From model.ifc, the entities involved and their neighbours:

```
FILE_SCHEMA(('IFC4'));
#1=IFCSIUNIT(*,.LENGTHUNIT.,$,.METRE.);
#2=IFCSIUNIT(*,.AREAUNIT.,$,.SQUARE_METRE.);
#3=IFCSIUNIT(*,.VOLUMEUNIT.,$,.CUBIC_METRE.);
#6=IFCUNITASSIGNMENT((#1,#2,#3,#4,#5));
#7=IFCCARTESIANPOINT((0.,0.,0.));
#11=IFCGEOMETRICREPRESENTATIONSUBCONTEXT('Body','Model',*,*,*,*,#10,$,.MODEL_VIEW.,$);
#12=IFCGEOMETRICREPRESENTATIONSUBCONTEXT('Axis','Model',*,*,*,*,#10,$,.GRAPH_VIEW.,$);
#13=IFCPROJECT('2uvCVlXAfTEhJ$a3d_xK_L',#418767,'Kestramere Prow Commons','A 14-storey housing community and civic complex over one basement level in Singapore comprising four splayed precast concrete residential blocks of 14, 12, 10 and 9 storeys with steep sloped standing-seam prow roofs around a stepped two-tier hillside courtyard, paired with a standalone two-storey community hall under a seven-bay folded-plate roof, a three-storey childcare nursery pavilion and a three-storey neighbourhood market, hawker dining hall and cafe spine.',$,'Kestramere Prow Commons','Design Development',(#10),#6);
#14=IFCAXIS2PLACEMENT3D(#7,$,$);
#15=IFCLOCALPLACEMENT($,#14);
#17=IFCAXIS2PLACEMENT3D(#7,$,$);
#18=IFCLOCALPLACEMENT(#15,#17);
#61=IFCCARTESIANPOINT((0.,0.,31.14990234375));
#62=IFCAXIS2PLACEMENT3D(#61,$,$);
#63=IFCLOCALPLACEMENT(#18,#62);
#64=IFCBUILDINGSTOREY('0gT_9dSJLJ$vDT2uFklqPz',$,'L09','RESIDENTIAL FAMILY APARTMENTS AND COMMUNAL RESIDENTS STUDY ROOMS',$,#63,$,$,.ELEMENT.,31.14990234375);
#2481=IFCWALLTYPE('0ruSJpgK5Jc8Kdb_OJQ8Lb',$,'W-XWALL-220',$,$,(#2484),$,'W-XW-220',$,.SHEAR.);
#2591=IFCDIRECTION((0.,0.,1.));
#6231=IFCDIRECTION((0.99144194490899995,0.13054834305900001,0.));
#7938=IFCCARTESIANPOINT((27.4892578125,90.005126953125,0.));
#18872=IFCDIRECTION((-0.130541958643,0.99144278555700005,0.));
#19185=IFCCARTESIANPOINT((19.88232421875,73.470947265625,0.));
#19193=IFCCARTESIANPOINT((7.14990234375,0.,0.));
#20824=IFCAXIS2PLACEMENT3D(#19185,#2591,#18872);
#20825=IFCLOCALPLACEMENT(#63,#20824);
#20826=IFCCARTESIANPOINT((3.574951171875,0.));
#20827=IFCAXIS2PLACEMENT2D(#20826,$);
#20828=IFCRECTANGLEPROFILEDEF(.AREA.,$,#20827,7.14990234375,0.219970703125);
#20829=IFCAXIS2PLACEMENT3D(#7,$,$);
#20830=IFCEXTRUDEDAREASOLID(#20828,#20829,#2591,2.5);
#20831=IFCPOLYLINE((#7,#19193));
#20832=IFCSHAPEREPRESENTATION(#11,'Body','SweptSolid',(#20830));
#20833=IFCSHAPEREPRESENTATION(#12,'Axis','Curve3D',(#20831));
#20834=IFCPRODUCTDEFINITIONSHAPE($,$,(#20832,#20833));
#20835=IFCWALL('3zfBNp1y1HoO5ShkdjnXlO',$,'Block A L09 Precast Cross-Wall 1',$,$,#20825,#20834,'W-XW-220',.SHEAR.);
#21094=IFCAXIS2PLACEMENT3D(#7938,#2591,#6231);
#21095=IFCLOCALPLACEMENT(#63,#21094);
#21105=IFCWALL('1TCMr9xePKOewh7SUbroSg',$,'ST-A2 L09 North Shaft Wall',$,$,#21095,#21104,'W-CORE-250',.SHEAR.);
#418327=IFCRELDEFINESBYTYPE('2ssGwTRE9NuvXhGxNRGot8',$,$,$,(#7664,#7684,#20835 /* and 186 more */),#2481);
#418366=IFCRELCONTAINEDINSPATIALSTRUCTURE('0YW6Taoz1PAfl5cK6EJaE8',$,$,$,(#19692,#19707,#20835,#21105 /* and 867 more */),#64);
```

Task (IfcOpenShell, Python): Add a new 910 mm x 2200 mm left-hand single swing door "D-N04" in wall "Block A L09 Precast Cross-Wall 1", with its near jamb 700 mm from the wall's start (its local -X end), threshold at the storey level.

```python
import numpy as np
import ifcopenshell
import ifcopenshell.api.feature
import ifcopenshell.api.geometry
import ifcopenshell.api.root
import ifcopenshell.api.spatial
import ifcopenshell.geom
import ifcopenshell.util.element
import ifcopenshell.util.placement
import ifcopenshell.util.representation
import ifcopenshell.util.shape
import ifcopenshell.util.unit

model = ifcopenshell.open("model.ifc")
unit_scale = ifcopenshell.util.unit.calculate_unit_scale(model)
settings = ifcopenshell.geom.settings()


def volume(element):
    """Net volume in cubic metres, openings subtracted."""
    shape = ifcopenshell.geom.create_shape(settings, element)
    return ifcopenshell.util.shape.get_volume(shape.geometry)


wall = model.by_id(20835)
storey = ifcopenshell.util.element.get_container(wall, ifc_class="IfcBuildingStorey")
context = ifcopenshell.util.representation.get_context(model, "Model", "Body", "MODEL_VIEW")
before = volume(wall)

width, height, from_end, sill = 0.91, 2.2, 0.7, 0.0  # metres

# The wall runs along its own X axis, and the end named is its -X end.
wall_shape = ifcopenshell.geom.create_shape(settings, wall)
x, y, z = ifcopenshell.util.shape.get_vertices(wall_shape.geometry).T
start = x.min() + from_end
face, thickness = float(y.min()), float(y.max() - y.min())
wall_matrix = ifcopenshell.util.placement.get_local_placement(wall.ObjectPlacement)
level = ifcopenshell.util.placement.get_local_placement(storey.ObjectPlacement)[2, 3]


def in_wall(x, y):
    """Placement at x, y metres in the wall's axes, at sill height."""
    matrix = wall_matrix.copy()
    matrix[:, 3] = wall_matrix @ np.array([x / unit_scale, y / unit_scale, 0.0, 1.0])
    matrix[2, 3] = level + sill / unit_scale
    return matrix


# Opening: a box that overshoots both wall faces by 50 mm.
opening = ifcopenshell.api.root.create_entity(model, ifc_class="IfcOpeningElement", predefined_type="OPENING")
box = ifcopenshell.api.geometry.add_wall_representation(
    model, context=context, length=width, height=height, thickness=thickness + 0.1
)
ifcopenshell.api.geometry.assign_representation(model, product=opening, representation=box)
ifcopenshell.api.geometry.edit_object_placement(model, product=opening, matrix=in_wall(start, face - 0.05), is_si=False)
ifcopenshell.api.feature.add_feature(model, feature=opening, element=wall)

door = ifcopenshell.api.root.create_entity(model, ifc_class="IfcDoor", name="D-N04", predefined_type="DOOR")
door.OverallWidth, door.OverallHeight = width / unit_scale, height / unit_scale
door.OperationType = "SINGLE_SWING_LEFT"
body = ifcopenshell.api.geometry.add_door_representation(
    model,
    context=context,
    overall_width=door.OverallWidth,
    overall_height=door.OverallHeight,
    operation_type="SINGLE_SWING_LEFT",
    lining_properties={"LiningDepth": thickness / unit_scale, "ThresholdDepth": thickness / unit_scale},
)
ifcopenshell.api.geometry.assign_representation(model, product=door, representation=body)
ifcopenshell.api.spatial.assign_container(model, products=[door], relating_structure=storey)
ifcopenshell.api.feature.add_filling(model, opening=opening, element=door)

# The lining spans the wall, so the door starts at the wall face.
ifcopenshell.api.geometry.edit_object_placement(model, product=door, matrix=in_wall(start, face), is_si=False)

after = volume(wall)

print(f"wall volume {before:.3f} -> {after:.3f} m3")

model.write("model_edited.ifc")
```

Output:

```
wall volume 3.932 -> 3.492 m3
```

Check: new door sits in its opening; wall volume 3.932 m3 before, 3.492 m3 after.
